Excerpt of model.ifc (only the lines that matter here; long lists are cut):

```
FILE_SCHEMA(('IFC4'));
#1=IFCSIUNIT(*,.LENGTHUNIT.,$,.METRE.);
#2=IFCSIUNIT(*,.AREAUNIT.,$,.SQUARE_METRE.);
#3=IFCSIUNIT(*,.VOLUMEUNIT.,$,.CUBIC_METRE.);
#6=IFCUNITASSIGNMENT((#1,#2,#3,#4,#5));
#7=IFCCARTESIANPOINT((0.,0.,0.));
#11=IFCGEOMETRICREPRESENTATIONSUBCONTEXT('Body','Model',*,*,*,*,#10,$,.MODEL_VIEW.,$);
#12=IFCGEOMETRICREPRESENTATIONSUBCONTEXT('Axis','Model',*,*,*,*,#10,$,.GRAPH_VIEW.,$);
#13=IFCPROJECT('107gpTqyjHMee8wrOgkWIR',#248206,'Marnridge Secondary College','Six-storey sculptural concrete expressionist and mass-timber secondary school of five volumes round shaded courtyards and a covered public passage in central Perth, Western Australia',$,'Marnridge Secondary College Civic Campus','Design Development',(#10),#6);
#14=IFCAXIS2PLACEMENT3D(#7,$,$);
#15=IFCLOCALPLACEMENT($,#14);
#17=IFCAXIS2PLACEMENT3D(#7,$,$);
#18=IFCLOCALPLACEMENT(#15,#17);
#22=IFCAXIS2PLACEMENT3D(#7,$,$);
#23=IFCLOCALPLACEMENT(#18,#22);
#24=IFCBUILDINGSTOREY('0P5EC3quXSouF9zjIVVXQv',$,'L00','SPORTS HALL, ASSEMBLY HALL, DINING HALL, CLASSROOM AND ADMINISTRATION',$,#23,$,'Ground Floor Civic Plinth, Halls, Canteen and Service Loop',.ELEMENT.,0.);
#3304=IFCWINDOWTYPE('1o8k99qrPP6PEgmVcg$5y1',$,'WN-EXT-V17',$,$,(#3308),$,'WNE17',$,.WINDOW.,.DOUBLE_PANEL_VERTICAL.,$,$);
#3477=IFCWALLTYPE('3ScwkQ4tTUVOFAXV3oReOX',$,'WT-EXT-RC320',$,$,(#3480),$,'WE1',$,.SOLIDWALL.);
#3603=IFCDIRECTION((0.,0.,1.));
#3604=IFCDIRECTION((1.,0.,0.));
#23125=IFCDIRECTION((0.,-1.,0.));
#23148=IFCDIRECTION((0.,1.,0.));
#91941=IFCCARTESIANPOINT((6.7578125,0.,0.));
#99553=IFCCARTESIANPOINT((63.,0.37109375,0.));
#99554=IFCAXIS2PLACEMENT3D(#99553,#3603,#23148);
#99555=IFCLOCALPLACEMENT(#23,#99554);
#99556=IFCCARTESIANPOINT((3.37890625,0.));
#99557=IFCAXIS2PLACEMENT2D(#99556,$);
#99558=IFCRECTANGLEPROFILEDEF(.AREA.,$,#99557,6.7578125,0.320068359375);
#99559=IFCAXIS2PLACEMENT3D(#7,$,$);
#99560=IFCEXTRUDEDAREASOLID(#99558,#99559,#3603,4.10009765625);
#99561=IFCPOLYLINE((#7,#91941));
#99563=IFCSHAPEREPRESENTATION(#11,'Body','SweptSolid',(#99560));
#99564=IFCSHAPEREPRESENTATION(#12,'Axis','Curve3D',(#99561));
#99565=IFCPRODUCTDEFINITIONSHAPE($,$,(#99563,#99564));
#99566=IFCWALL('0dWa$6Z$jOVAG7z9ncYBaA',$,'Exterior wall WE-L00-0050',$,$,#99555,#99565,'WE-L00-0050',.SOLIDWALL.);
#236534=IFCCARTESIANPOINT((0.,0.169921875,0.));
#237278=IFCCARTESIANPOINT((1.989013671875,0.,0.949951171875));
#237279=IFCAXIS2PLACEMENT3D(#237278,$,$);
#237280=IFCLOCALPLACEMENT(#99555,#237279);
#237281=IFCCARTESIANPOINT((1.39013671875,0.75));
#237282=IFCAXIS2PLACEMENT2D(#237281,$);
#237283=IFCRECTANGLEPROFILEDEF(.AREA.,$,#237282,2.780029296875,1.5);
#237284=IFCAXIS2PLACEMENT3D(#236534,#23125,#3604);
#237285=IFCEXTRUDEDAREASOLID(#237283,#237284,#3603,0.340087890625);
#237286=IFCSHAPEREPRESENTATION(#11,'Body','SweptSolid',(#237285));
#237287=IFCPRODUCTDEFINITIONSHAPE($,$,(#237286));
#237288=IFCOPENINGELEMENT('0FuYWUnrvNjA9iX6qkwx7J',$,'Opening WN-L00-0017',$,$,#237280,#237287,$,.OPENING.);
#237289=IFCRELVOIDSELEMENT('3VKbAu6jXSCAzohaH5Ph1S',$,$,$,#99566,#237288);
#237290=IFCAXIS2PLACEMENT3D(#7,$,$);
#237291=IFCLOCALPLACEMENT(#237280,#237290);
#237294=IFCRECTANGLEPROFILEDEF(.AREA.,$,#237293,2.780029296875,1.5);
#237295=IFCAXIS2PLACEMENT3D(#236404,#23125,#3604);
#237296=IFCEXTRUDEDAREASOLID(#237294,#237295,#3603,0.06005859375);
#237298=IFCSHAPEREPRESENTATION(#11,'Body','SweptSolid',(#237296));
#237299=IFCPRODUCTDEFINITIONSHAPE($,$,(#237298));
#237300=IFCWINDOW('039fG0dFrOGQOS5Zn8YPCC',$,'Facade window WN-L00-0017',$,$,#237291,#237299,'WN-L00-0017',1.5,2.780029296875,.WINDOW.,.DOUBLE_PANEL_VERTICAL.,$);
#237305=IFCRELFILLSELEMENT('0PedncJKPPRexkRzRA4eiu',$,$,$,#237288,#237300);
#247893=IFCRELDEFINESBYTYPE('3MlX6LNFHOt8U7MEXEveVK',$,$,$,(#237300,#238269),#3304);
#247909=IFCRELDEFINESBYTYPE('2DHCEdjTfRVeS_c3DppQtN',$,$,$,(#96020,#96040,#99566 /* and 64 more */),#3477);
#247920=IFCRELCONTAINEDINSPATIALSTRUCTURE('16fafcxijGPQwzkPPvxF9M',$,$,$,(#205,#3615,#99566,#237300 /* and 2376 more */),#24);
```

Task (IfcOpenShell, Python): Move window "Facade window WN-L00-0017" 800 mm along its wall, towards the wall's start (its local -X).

```python
import ifcopenshell
import ifcopenshell.api.geometry
import ifcopenshell.util.placement
import ifcopenshell.util.unit

model = ifcopenshell.open("model.ifc")
unit_scale = ifcopenshell.util.unit.calculate_unit_scale(model)

window = model.by_guid("039fG0dFrOGQOS5Zn8YPCC")
opening = window.FillsVoids[0].RelatingOpeningElement
wall = opening.VoidsElements[0].RelatingBuildingElement

wall_matrix = ifcopenshell.util.placement.get_local_placement(wall.ObjectPlacement)
shift = wall_matrix[:3, 0] * -0.8 / unit_scale
before = ifcopenshell.util.placement.get_local_placement(window.ObjectPlacement)[:3, 3].copy()

# The window is placed relative to its opening, so it follows when the opening moves.
matrix = ifcopenshell.util.placement.get_local_placement(opening.ObjectPlacement)
matrix[:3, 3] += shift
ifcopenshell.api.geometry.edit_object_placement(
    model, product=opening, matrix=matrix, is_si=False, should_transform_children=True
)

after = ifcopenshell.util.placement.get_local_placement(window.ObjectPlacement)[:3, 3]
print("window moved by", (after - before).round(3) + 0.0)

model.write("model_edited.ifc")
```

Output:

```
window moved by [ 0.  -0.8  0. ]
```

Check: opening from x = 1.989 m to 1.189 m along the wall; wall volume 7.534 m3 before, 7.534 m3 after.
